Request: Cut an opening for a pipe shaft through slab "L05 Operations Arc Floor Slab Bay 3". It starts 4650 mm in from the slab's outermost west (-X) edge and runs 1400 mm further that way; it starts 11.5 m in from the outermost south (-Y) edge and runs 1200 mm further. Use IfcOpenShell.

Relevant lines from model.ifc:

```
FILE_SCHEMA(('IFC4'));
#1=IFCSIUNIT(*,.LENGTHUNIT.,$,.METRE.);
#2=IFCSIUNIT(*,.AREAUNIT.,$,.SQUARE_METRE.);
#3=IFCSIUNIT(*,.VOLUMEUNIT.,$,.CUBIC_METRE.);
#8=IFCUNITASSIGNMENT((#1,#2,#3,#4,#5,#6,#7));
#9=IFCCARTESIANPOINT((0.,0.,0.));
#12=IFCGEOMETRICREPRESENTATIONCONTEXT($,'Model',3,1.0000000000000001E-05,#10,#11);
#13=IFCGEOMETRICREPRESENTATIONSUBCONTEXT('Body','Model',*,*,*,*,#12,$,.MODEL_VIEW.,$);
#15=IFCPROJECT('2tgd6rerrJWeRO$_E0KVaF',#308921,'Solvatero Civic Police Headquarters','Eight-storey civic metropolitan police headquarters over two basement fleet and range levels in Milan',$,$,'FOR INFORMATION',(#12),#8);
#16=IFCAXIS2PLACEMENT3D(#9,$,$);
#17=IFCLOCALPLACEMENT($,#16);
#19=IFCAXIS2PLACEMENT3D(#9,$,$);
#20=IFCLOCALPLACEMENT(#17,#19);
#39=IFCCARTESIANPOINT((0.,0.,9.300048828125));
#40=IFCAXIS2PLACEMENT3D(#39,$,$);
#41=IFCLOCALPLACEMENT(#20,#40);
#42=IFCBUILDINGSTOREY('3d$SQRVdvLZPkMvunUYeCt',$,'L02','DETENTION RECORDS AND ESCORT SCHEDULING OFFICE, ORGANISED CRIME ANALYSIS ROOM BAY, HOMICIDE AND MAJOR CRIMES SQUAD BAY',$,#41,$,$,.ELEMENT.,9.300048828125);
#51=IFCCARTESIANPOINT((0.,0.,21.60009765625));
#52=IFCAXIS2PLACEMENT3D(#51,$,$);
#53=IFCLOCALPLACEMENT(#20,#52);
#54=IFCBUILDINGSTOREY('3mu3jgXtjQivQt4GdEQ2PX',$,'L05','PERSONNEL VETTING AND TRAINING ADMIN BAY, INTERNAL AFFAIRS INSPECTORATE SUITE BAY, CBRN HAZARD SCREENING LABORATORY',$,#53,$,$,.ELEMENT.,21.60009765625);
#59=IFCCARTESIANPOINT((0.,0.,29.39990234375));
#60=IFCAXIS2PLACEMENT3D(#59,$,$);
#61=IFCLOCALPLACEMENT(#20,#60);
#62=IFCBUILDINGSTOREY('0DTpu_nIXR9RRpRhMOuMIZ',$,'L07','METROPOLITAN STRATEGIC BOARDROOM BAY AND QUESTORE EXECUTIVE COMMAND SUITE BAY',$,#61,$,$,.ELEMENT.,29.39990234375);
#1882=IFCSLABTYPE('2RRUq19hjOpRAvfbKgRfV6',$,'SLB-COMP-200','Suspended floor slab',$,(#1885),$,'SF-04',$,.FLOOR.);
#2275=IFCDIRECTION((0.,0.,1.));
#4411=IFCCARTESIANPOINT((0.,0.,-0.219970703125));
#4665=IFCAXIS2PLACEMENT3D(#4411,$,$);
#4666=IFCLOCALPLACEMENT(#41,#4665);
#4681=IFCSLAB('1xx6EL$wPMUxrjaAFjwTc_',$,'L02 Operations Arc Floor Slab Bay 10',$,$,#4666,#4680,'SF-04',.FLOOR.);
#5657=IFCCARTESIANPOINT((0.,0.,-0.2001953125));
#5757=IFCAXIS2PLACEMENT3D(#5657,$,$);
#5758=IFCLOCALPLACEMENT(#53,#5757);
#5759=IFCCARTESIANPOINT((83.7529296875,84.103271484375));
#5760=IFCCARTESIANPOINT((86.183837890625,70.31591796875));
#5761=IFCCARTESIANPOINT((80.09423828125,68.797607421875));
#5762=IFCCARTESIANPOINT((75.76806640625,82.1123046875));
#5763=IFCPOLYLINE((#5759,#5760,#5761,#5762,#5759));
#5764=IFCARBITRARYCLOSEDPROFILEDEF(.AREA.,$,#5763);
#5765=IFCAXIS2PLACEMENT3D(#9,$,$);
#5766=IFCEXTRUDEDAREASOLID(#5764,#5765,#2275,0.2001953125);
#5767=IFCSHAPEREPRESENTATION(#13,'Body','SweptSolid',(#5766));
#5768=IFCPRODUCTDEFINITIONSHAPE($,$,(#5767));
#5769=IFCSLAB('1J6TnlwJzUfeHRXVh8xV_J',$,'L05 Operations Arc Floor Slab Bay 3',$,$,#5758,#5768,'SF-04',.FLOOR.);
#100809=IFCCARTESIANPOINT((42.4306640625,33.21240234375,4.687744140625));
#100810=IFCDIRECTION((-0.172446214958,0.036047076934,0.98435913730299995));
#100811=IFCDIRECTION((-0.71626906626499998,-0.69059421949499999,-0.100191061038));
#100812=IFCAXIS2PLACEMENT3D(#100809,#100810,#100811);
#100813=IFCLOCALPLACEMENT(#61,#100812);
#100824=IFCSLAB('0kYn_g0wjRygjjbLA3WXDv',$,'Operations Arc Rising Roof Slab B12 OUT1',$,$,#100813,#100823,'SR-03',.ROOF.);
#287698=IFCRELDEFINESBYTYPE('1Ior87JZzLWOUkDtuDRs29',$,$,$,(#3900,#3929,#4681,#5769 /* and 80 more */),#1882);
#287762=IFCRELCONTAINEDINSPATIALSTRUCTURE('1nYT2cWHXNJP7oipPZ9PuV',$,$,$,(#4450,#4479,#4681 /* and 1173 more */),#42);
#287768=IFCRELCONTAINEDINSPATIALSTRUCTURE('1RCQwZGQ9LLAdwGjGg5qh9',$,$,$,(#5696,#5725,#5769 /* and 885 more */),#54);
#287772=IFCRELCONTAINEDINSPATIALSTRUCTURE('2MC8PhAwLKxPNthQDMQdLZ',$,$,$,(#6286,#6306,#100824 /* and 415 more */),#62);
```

```python
import numpy as np
import ifcopenshell
import ifcopenshell.api.feature
import ifcopenshell.api.geometry
import ifcopenshell.api.root
import ifcopenshell.geom
import ifcopenshell.util.placement
import ifcopenshell.util.representation
import ifcopenshell.util.shape
import ifcopenshell.util.unit

model = ifcopenshell.open("model.ifc")
unit_scale = ifcopenshell.util.unit.calculate_unit_scale(model)
settings = ifcopenshell.geom.settings()


def volume(element):
    """Net volume in cubic metres, openings subtracted."""
    shape = ifcopenshell.geom.create_shape(settings, element)
    return ifcopenshell.util.shape.get_volume(shape.geometry)


slab = model.by_guid("1J6TnlwJzUfeHRXVh8xV_J")
before = volume(slab)

# Extent in the slab's own axes, in metres. The edges named are its -X and -Y sides.
slab_shape = ifcopenshell.geom.create_shape(settings, slab)
vertices = ifcopenshell.util.shape.get_vertices(slab_shape.geometry)
x_min, y_min, bottom = vertices.min(axis=0)
top = vertices[:, 2].max()

opening = ifcopenshell.api.root.create_entity(model, ifc_class="IfcOpeningElement", name="Pipe shaft opening", predefined_type="OPENING")
context = ifcopenshell.util.representation.get_context(model, "Model", "Body", "MODEL_VIEW")
width, depth = 1.4, 1.2
outline = [(0.0, 0.0), (width, 0.0), (width, depth), (0.0, depth), (0.0, 0.0)]
# Overshoot both faces by 50 mm so the cut is clean.
shape = ifcopenshell.api.geometry.add_slab_representation(
    model, context=context, depth=top - bottom + 0.1, polyline=outline
)
ifcopenshell.api.geometry.assign_representation(model, product=opening, representation=shape)

matrix = ifcopenshell.util.placement.get_local_placement(slab.ObjectPlacement)
matrix[:, 3] = matrix @ np.append(np.array([x_min + 4.65, y_min + 11.5, bottom - 0.05]) / unit_scale, 1.0)
ifcopenshell.api.geometry.edit_object_placement(model, product=opening, matrix=matrix, is_si=False)
ifcopenshell.api.feature.add_feature(model, feature=opening, element=slab)

after = volume(slab)

print(f"slab volume {before:.3f} -> {after:.3f} m3")

model.write("model_updated.ifc")
```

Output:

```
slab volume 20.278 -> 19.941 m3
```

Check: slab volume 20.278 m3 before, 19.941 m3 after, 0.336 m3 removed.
